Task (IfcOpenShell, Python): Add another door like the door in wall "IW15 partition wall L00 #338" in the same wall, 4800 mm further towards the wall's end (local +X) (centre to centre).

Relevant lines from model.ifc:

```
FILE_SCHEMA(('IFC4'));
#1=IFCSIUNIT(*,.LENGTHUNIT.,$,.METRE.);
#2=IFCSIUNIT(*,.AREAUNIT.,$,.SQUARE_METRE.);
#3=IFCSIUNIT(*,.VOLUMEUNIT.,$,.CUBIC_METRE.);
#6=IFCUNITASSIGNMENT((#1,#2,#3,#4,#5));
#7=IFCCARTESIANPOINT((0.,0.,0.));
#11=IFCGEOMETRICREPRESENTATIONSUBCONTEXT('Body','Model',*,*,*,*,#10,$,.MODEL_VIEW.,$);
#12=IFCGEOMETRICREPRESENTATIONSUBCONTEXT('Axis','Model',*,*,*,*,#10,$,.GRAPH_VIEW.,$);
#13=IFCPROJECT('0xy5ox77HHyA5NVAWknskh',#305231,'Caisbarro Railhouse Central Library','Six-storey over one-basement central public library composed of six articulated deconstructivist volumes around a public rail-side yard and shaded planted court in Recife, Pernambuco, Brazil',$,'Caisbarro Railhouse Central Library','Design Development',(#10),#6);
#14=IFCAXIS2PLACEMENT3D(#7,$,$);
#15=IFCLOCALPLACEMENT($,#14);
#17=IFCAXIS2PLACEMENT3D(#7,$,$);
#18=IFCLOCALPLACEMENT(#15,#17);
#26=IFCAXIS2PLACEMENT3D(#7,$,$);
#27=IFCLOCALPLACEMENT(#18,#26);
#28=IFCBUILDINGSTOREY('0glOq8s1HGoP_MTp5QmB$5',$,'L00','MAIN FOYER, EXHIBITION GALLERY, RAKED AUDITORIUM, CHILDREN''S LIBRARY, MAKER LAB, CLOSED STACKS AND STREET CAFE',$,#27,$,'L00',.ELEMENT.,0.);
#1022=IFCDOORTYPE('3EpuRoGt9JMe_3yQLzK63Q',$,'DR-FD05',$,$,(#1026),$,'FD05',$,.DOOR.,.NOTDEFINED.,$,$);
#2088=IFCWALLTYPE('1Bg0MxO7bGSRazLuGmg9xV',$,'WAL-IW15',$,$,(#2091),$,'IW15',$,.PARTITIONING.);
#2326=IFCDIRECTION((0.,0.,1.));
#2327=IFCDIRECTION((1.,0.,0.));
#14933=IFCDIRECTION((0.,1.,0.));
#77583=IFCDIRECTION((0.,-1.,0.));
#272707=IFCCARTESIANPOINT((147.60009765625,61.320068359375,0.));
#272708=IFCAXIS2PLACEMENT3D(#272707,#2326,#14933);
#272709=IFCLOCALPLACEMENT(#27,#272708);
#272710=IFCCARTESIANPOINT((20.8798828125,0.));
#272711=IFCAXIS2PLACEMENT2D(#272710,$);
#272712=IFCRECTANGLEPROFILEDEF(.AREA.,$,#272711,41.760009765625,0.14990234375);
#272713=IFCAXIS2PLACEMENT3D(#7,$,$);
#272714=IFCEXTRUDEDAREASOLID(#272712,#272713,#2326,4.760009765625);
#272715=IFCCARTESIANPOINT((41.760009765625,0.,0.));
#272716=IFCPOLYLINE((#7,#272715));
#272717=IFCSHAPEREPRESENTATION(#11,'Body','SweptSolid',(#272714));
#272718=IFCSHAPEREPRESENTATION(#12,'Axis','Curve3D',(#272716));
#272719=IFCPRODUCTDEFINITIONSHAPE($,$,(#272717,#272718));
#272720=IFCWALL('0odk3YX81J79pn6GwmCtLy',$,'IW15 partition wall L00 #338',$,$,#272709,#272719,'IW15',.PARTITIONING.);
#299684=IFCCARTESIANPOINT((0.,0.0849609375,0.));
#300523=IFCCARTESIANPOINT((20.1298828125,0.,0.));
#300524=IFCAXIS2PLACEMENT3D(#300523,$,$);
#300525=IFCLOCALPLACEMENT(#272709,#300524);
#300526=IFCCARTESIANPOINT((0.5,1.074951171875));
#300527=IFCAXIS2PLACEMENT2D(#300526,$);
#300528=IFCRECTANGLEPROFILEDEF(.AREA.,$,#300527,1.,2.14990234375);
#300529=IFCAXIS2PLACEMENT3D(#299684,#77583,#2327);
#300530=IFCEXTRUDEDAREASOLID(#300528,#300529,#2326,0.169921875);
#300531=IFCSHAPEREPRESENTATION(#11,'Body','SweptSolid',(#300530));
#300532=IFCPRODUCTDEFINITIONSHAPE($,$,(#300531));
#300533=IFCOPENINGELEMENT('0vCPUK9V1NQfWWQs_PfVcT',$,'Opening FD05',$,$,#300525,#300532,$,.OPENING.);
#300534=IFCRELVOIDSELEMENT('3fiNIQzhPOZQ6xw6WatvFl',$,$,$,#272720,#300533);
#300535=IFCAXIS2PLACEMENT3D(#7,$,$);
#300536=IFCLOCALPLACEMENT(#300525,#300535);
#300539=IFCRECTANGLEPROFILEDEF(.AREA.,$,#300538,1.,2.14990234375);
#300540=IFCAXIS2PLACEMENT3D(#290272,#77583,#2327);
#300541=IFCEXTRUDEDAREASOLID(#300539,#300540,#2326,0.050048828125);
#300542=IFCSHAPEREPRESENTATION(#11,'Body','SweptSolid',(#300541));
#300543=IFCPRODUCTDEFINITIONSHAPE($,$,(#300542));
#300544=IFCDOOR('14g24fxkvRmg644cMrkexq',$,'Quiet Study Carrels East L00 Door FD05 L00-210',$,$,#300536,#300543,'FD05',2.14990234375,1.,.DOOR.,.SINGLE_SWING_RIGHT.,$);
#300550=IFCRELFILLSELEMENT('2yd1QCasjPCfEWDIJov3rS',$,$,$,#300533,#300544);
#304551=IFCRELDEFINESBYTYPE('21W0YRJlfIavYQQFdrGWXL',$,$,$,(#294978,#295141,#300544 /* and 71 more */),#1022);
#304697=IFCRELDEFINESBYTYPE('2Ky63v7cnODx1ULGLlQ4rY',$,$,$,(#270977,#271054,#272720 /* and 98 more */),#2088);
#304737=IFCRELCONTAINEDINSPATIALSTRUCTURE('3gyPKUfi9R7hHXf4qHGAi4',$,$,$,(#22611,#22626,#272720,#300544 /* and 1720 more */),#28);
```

```python
import ifcopenshell
import ifcopenshell.api.feature
import ifcopenshell.api.geometry
import ifcopenshell.api.root
import ifcopenshell.geom
import ifcopenshell.util.element
import ifcopenshell.util.placement
import ifcopenshell.util.shape

model = ifcopenshell.open("model.ifc")
settings = ifcopenshell.geom.settings()


def volume(element):
    """Net volume in cubic metres, openings subtracted."""
    shape = ifcopenshell.geom.create_shape(settings, element)
    return ifcopenshell.util.shape.get_volume(shape.geometry)


door = model.by_id(300544)
opening = door.FillsVoids[0].RelatingOpeningElement
wall = opening.VoidsElements[0].RelatingBuildingElement
before = volume(wall)
shift = ifcopenshell.util.placement.get_local_placement(wall.ObjectPlacement)[:3, 0] * 4.8

# copy_class copies the void relationship, type, container and properties, but no geometry.
new_opening = ifcopenshell.api.root.copy_class(model, product=opening)
new_opening.Representation = ifcopenshell.util.element.copy_deep(
    model, opening.Representation, exclude=["IfcGeometricRepresentationContext", "IfcRepresentationMap"]
)
new_door = ifcopenshell.api.root.copy_class(model, product=door)
new_door.Representation = ifcopenshell.util.element.copy_deep(
    model, door.Representation, exclude=["IfcGeometricRepresentationContext", "IfcRepresentationMap"]
)
new_door.Tag = None
ifcopenshell.api.feature.add_filling(model, opening=new_opening, element=new_door)

for old, new in ((opening, new_opening), (door, new_door)):
    matrix = ifcopenshell.util.placement.get_local_placement(old.ObjectPlacement)
    matrix[:3, 3] += shift
    ifcopenshell.api.geometry.edit_object_placement(model, product=new, matrix=matrix, is_si=False)

after = volume(wall)

print(f"wall volume {before:.3f} -> {after:.3f} m3")

model.write("model_edited.ifc")
```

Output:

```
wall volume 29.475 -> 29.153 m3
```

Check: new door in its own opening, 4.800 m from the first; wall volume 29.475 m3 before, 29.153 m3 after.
